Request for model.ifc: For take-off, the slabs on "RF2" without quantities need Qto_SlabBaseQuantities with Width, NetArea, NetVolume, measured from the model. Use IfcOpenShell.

First a look at what the model holds.

```python
import ifcopenshell
import ifcopenshell.util.element
import ifcopenshell.util.unit

model = ifcopenshell.open("model.ifc")
print(model.schema)
for unit_type in ("LENGTHUNIT", "AREAUNIT", "VOLUMEUNIT"):
    print(unit_type, ifcopenshell.util.unit.calculate_unit_scale(model, unit_type))
storey = next(s for s in model.by_type("IfcBuildingStorey") if s.Name == "RF2")
slabs = [e for e in ifcopenshell.util.element.get_decomposition(storey) if e.is_a("IfcSlab")]
for e in sorted(slabs, key=lambda e: e.id()):
    print(e.id(), e.is_a(), e.Name, list(ifcopenshell.util.element.get_psets(e, qtos_only=True)), sep=" | ")
```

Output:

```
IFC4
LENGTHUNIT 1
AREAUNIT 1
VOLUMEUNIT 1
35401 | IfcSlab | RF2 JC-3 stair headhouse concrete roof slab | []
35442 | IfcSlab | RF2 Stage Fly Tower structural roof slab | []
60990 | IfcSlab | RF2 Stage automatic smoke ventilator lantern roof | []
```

```python
import ifcopenshell
import ifcopenshell.api.pset
import ifcopenshell.geom
import ifcopenshell.util.element
import ifcopenshell.util.shape
import ifcopenshell.util.unit

model = ifcopenshell.open("model.ifc")
unit_scale = ifcopenshell.util.unit.calculate_unit_scale(model)
area_scale = ifcopenshell.util.unit.calculate_unit_scale(model, "AREAUNIT")
volume_scale = ifcopenshell.util.unit.calculate_unit_scale(model, "VOLUMEUNIT")
settings = ifcopenshell.geom.settings()

storey = next(s for s in model.by_type("IfcBuildingStorey") if s.Name == "RF2")
slabs = [e for e in ifcopenshell.util.element.get_decomposition(storey) if e.is_a("IfcSlab")]

for e in sorted(slabs, key=lambda e: e.id()):
    if ifcopenshell.util.element.get_psets(e, qtos_only=True, should_inherit=False):
        continue
    # Geometry comes back in metres, in the element's own axes.
    shape = ifcopenshell.geom.create_shape(settings, e)
    values = {
        "Width": ifcopenshell.util.shape.get_z(shape.geometry) / unit_scale,
        "NetArea": ifcopenshell.util.shape.get_footprint_area(shape.geometry) / area_scale,
        "NetVolume": ifcopenshell.util.shape.get_volume(shape.geometry) / volume_scale,
    }
    qto = ifcopenshell.api.pset.add_qto(model, product=e, name="Qto_SlabBaseQuantities")
    ifcopenshell.api.pset.edit_qto(model, qto=qto, properties=values)
    print(e.id(), {k: round(v, 3) for k, v in values.items()})

model.write("model_updated.ifc")
```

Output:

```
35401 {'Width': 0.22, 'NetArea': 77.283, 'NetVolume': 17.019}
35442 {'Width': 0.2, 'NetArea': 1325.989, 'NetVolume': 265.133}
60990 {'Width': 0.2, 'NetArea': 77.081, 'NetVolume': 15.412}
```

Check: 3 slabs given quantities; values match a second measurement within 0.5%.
